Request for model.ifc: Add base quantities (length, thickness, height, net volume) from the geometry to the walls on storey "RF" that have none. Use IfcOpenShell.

First a look at what the model holds.

```python
import ifcopenshell
import ifcopenshell.util.element
import ifcopenshell.util.unit

model = ifcopenshell.open("model.ifc")
print(model.schema)
for unit_type in ("LENGTHUNIT", "AREAUNIT", "VOLUMEUNIT"):
    print(unit_type, ifcopenshell.util.unit.calculate_unit_scale(model, unit_type))
storey = next(s for s in model.by_type("IfcBuildingStorey") if s.Name == "RF")
walls = [e for e in ifcopenshell.util.element.get_decomposition(storey) if e.is_a("IfcWall")]
for e in sorted(walls, key=lambda e: e.id()):
    print(e.id(), e.is_a(), e.Name, list(ifcopenshell.util.element.get_psets(e, qtos_only=True)), sep=" | ")
```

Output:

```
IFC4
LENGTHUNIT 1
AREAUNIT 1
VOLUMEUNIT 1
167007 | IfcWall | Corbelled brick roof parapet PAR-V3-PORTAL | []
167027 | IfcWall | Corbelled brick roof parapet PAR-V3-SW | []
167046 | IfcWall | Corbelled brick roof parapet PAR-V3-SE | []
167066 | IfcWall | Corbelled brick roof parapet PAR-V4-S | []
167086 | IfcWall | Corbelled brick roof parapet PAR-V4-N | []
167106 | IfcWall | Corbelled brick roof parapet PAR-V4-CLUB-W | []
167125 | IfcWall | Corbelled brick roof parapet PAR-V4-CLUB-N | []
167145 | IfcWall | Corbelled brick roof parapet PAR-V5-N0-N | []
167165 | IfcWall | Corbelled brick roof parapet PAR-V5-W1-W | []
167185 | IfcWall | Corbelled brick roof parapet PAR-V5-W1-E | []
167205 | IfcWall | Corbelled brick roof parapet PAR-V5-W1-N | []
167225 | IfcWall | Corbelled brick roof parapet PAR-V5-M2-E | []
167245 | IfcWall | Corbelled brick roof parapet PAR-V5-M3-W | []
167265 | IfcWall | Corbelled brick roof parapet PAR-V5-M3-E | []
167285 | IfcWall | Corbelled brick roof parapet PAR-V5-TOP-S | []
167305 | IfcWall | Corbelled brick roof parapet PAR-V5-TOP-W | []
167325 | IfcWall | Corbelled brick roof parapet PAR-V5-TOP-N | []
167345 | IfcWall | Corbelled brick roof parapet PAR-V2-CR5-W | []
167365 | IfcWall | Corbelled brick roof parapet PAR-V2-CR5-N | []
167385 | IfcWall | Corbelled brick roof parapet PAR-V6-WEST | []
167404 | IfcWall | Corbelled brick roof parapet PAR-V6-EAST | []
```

```python
import ifcopenshell
import ifcopenshell.api.pset
import ifcopenshell.geom
import ifcopenshell.util.element
import ifcopenshell.util.shape
import ifcopenshell.util.unit

model = ifcopenshell.open("model.ifc")
unit_scale = ifcopenshell.util.unit.calculate_unit_scale(model)
volume_scale = ifcopenshell.util.unit.calculate_unit_scale(model, "VOLUMEUNIT")
settings = ifcopenshell.geom.settings()

storey = next(s for s in model.by_type("IfcBuildingStorey") if s.Name == "RF")
walls = [e for e in ifcopenshell.util.element.get_decomposition(storey) if e.is_a("IfcWall")]

for e in sorted(walls, key=lambda e: e.id()):
    if ifcopenshell.util.element.get_psets(e, qtos_only=True, should_inherit=False):
        continue
    # Geometry comes back in metres, in the element's own axes.
    shape = ifcopenshell.geom.create_shape(settings, e)
    values = {
        "Length": ifcopenshell.util.shape.get_x(shape.geometry) / unit_scale,
        "Width": ifcopenshell.util.shape.get_y(shape.geometry) / unit_scale,
        "Height": ifcopenshell.util.shape.get_z(shape.geometry) / unit_scale,
        "NetVolume": ifcopenshell.util.shape.get_volume(shape.geometry) / volume_scale,
    }
    qto = ifcopenshell.api.pset.add_qto(model, product=e, name="Qto_WallBaseQuantities")
    ifcopenshell.api.pset.edit_qto(model, qto=qto, properties=values)
    print(e.id(), {k: round(v, 3) for k, v in values.items()})

model.write("model_rev.ifc")
```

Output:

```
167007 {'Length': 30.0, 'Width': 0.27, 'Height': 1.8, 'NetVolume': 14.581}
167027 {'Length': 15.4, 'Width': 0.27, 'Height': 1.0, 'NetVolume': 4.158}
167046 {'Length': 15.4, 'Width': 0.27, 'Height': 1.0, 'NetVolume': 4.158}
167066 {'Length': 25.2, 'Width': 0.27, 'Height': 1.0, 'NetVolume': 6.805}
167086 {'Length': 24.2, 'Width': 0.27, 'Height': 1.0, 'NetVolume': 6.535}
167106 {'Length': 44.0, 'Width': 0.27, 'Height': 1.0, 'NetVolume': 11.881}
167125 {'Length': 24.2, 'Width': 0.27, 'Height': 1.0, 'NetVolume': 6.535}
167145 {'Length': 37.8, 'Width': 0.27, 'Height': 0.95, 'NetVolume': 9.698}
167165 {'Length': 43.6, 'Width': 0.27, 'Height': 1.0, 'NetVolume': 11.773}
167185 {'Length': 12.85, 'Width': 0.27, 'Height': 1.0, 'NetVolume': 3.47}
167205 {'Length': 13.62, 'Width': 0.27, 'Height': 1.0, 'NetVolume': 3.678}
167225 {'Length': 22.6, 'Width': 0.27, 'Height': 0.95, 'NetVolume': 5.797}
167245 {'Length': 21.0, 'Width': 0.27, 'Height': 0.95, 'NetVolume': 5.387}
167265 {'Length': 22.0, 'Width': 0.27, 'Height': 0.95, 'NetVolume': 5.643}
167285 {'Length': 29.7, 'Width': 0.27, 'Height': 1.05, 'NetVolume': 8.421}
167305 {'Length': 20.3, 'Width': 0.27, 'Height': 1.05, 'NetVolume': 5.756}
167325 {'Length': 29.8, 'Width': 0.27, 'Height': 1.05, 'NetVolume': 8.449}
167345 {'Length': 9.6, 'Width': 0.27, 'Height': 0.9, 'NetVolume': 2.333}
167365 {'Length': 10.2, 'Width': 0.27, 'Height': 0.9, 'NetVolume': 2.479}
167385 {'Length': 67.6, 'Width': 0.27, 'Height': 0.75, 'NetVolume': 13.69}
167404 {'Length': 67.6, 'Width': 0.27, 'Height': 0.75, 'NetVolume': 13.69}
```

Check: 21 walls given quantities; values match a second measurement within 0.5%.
